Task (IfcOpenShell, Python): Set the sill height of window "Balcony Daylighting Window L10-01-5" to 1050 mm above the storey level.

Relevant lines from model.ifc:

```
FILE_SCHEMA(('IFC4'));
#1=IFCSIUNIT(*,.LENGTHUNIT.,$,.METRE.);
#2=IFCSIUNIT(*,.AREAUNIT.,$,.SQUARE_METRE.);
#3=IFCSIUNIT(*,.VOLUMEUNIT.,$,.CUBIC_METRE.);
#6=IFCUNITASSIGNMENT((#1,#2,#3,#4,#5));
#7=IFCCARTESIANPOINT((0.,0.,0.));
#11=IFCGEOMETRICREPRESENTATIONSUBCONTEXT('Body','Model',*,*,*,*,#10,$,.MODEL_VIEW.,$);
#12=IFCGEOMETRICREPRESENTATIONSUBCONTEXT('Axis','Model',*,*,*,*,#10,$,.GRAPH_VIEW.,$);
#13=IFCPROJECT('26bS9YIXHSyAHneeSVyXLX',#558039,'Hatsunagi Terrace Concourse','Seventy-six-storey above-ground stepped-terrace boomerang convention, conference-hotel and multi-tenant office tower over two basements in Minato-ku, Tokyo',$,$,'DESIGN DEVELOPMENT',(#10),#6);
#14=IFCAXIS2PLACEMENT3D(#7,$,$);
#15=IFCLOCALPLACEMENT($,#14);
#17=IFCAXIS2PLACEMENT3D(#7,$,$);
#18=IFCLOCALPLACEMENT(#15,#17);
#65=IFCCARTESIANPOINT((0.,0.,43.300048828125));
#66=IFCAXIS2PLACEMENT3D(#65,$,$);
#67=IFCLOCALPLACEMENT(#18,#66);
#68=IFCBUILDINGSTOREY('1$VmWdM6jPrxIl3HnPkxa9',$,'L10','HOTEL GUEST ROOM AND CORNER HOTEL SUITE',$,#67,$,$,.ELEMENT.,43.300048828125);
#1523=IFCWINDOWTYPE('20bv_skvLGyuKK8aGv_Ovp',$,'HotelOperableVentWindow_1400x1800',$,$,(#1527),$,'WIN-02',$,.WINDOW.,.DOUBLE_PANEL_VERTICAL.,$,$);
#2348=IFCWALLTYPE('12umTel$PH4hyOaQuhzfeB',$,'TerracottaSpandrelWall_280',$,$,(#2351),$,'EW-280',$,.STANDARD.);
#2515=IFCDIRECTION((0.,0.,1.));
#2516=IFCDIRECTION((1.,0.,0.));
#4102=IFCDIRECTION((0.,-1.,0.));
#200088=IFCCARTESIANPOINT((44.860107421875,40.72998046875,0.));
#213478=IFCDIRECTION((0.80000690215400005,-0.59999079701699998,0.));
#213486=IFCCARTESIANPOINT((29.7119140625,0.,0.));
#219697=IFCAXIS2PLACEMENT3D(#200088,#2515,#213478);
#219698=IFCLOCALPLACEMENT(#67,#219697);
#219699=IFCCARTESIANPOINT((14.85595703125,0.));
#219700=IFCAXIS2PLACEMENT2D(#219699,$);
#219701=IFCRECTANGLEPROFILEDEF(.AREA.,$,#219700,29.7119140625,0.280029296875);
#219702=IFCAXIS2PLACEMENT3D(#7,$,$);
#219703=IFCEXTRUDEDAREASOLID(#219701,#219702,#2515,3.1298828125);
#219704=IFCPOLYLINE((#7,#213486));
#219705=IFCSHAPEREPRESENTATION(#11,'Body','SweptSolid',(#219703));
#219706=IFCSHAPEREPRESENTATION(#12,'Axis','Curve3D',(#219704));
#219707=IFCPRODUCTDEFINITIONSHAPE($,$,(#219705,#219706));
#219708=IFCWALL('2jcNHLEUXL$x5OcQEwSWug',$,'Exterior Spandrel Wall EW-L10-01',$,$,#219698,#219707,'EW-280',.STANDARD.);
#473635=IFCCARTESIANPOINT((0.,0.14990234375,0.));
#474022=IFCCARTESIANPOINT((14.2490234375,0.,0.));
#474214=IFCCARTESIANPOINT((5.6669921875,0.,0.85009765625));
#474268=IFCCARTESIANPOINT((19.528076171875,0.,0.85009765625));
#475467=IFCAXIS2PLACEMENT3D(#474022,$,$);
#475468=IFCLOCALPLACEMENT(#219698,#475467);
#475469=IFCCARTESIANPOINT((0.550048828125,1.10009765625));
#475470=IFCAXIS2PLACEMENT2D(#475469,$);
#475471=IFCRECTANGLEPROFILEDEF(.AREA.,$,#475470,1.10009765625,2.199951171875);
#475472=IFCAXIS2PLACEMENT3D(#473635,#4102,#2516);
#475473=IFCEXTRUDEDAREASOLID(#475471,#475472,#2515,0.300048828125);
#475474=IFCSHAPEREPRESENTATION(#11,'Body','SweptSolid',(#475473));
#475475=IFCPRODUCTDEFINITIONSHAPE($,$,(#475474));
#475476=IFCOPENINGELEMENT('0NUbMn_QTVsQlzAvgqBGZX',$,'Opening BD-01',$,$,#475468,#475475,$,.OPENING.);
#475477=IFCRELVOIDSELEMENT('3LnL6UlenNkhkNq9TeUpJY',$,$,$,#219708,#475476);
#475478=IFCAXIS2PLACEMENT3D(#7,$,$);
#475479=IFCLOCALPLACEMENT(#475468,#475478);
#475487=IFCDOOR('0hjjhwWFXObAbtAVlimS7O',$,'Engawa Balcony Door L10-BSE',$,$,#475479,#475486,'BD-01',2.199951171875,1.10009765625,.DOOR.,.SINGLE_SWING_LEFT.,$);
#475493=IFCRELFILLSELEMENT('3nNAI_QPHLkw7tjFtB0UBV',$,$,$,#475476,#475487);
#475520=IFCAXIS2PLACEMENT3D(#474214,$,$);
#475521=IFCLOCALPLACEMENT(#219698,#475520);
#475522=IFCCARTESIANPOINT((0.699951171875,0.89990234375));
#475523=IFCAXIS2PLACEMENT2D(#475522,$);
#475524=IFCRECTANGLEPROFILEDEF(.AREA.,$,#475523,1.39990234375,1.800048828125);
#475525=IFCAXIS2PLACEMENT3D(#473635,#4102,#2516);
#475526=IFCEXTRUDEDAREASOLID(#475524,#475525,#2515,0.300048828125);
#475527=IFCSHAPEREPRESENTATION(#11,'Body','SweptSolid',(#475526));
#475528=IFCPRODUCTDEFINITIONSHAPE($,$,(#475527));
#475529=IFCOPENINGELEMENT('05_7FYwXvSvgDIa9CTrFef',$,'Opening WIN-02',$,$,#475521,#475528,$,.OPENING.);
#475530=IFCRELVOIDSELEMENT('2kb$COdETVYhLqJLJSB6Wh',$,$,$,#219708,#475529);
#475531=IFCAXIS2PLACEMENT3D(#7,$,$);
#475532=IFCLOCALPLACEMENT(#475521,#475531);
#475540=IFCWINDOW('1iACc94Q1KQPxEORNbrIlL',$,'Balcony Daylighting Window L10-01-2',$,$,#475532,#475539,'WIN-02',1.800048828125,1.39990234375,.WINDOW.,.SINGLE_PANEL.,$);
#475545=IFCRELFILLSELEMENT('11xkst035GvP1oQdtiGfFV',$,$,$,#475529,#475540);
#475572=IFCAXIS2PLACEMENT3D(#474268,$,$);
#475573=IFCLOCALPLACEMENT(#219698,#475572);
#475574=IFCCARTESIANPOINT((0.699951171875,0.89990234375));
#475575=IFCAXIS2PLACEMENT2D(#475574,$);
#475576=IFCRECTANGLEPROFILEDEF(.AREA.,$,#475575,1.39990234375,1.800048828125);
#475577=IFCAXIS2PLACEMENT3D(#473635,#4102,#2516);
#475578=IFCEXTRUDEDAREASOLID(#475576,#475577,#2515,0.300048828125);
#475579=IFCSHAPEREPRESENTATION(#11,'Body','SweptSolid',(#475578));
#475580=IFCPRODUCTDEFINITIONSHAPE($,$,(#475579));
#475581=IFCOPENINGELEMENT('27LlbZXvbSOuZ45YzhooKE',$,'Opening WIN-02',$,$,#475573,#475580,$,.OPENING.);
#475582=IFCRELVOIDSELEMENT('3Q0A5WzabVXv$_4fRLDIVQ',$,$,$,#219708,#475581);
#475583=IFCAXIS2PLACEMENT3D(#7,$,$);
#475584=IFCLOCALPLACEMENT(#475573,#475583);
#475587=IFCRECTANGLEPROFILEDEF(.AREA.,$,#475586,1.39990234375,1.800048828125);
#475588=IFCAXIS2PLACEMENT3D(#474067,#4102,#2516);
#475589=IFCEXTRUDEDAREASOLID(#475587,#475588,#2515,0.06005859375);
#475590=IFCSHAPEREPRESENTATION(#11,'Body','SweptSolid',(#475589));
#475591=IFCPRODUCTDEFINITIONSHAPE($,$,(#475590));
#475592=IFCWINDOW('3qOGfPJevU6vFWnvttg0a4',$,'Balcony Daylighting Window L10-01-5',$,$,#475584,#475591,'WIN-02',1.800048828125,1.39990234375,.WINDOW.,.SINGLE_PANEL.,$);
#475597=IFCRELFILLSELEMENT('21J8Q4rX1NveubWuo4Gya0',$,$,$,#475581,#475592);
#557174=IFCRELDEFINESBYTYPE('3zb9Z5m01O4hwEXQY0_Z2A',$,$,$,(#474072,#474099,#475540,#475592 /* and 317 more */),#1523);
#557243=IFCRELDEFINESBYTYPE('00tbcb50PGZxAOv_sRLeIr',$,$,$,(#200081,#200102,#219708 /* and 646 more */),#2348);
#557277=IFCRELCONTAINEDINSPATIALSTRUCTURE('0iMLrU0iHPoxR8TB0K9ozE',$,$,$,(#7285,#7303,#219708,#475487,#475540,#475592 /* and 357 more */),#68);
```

```python
import numpy as np
import ifcopenshell
import ifcopenshell.api.geometry
import ifcopenshell.geom
import ifcopenshell.util.element
import ifcopenshell.util.placement
import ifcopenshell.util.shape
import ifcopenshell.util.unit

model = ifcopenshell.open("model.ifc")
unit_scale = ifcopenshell.util.unit.calculate_unit_scale(model)

window = model.by_id(475592)
opening = window.FillsVoids[0].RelatingOpeningElement
storey = ifcopenshell.util.element.get_container(window, ifc_class="IfcBuildingStorey")
level = ifcopenshell.util.placement.get_local_placement(storey.ObjectPlacement)[2, 3]

# The opening's origin need not be at the sill, so measure its lowest point.
shape = ifcopenshell.geom.create_shape(ifcopenshell.geom.settings(), opening)
bottom = ifcopenshell.util.shape.get_shape_bottom_elevation(shape, shape.geometry) / unit_scale
dz = level + 1.05 - bottom

shift = np.array([0.0, 0.0, dz])
# The window is placed relative to its opening, so it follows when the opening moves.
matrix = ifcopenshell.util.placement.get_local_placement(opening.ObjectPlacement)
matrix[:3, 3] += shift
ifcopenshell.api.geometry.edit_object_placement(
    model, product=opening, matrix=matrix, is_si=False, should_transform_children=True
)

print(f"moved by {dz * unit_scale:+.3f} m")

model.write("model-out.ifc")
```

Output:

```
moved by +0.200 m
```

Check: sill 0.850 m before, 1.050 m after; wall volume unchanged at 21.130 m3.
